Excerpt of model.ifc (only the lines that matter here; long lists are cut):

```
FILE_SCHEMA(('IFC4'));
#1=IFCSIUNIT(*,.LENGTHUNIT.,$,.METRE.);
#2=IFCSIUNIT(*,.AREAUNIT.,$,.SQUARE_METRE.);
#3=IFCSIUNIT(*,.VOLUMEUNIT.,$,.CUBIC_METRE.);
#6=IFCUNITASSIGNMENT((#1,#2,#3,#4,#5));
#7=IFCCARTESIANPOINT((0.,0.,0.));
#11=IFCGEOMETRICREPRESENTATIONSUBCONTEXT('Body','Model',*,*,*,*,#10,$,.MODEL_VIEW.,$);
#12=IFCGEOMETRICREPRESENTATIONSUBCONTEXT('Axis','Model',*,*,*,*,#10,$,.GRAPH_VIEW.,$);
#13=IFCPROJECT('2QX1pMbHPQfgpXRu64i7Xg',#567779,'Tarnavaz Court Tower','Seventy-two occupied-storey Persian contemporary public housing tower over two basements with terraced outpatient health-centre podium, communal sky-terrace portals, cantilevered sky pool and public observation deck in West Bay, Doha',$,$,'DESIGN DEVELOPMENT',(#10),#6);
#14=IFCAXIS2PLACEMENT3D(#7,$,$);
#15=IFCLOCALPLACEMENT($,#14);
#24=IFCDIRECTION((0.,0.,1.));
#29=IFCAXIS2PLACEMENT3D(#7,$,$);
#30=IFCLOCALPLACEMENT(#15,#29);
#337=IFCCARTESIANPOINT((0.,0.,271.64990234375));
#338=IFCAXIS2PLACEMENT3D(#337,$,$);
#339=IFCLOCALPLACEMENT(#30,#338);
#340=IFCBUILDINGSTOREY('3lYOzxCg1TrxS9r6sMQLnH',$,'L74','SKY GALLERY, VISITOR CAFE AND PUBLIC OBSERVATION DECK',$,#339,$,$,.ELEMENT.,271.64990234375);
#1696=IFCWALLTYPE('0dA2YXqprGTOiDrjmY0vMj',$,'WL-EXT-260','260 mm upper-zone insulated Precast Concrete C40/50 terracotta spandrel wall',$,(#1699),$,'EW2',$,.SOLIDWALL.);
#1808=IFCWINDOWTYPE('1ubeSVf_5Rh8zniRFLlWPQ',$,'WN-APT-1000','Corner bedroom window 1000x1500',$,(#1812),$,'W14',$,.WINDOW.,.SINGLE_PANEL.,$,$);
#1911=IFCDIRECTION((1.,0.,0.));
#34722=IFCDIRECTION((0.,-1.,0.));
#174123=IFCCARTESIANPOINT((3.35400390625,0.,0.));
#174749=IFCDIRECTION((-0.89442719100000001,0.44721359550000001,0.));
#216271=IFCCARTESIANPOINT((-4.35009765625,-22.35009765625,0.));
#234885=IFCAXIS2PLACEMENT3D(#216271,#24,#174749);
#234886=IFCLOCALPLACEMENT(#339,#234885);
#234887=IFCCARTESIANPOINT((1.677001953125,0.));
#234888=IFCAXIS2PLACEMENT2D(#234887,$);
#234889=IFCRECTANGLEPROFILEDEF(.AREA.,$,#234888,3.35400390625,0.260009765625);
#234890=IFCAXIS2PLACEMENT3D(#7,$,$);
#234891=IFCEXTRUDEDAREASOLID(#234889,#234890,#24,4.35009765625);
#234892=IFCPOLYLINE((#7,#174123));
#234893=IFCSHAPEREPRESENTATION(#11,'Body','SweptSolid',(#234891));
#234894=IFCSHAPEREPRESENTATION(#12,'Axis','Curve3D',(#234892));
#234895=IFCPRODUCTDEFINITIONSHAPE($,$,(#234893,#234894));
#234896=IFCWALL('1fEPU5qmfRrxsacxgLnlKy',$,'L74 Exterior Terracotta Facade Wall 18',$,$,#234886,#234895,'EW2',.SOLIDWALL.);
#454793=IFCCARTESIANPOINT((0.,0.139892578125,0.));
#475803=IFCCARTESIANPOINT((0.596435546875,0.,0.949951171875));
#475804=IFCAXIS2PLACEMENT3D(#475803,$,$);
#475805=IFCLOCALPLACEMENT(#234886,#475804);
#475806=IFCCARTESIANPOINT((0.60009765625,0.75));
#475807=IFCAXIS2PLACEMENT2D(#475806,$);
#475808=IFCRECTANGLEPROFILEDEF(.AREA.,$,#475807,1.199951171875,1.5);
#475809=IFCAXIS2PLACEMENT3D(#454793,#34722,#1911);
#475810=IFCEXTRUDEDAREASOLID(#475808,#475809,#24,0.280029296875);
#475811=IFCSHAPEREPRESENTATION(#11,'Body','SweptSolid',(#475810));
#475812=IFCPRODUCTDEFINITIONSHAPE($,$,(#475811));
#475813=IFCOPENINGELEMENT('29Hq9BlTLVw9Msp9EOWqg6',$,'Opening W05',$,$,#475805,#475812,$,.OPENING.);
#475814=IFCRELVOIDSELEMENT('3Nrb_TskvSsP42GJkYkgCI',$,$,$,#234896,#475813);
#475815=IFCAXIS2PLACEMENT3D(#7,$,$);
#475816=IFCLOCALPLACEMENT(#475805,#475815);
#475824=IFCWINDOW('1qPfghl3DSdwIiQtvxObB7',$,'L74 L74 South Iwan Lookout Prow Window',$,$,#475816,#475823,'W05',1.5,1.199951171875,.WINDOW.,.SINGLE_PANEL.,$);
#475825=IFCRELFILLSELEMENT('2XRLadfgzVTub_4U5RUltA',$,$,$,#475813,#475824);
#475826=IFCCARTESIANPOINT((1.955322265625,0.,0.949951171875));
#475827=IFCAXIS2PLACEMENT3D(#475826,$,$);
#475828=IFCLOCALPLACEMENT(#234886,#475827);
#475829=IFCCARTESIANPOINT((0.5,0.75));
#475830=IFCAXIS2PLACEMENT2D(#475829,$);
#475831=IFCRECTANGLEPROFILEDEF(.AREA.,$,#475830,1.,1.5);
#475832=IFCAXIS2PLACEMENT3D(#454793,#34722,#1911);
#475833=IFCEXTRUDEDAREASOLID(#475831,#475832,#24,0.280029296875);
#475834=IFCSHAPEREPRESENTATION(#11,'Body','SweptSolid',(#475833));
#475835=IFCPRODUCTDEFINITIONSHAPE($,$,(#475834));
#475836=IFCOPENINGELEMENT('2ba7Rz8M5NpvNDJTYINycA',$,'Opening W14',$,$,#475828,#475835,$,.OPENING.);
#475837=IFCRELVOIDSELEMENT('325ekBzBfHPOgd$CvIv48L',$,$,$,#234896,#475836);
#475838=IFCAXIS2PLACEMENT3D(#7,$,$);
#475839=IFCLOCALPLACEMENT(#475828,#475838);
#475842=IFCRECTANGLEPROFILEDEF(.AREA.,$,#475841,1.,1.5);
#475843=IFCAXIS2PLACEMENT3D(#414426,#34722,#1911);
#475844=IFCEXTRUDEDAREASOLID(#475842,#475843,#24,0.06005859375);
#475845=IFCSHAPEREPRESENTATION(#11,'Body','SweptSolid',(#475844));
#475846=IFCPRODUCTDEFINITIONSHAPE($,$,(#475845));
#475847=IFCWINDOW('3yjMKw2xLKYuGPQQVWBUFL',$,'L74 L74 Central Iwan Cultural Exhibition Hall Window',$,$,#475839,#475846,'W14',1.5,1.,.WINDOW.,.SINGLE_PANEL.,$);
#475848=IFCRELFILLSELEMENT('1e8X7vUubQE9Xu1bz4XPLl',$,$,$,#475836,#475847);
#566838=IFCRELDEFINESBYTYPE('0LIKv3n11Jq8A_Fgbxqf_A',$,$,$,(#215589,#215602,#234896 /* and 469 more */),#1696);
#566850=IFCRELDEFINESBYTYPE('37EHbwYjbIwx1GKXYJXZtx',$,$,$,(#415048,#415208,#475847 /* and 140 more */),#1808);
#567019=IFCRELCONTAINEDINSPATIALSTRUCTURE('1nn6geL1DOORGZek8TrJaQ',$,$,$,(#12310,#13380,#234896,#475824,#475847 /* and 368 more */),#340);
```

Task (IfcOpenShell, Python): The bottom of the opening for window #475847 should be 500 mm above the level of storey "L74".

```python
import numpy as np
import ifcopenshell
import ifcopenshell.api.geometry
import ifcopenshell.geom
import ifcopenshell.util.element
import ifcopenshell.util.placement
import ifcopenshell.util.shape
import ifcopenshell.util.unit

model = ifcopenshell.open("model.ifc")
unit_scale = ifcopenshell.util.unit.calculate_unit_scale(model)

window = model.by_id(475847)
opening = window.FillsVoids[0].RelatingOpeningElement
storey = ifcopenshell.util.element.get_container(window, ifc_class="IfcBuildingStorey")
level = ifcopenshell.util.placement.get_local_placement(storey.ObjectPlacement)[2, 3]

# The opening's origin need not be at the sill, so measure its lowest point.
shape = ifcopenshell.geom.create_shape(ifcopenshell.geom.settings(), opening)
bottom = ifcopenshell.util.shape.get_shape_bottom_elevation(shape, shape.geometry) / unit_scale
dz = level + 0.5 / unit_scale - bottom

shift = np.array([0.0, 0.0, dz])
# The window is placed relative to its opening, so it follows when the opening moves.
matrix = ifcopenshell.util.placement.get_local_placement(opening.ObjectPlacement)
matrix[:3, 3] += shift
ifcopenshell.api.geometry.edit_object_placement(
    model, product=opening, matrix=matrix, is_si=False, should_transform_children=True
)

print(f"moved by {dz * unit_scale:+.3f} m")

model.write("model_updated.ifc")
```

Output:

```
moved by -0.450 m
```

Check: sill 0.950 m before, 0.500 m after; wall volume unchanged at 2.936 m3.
